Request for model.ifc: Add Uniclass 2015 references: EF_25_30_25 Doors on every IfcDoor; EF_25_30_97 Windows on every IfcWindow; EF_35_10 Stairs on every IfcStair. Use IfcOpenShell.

First a look at what the model holds.

```python
import ifcopenshell

model = ifcopenshell.open("model.ifc")
print(model.schema)
print("classifications:", [c.Name for c in model.by_type("IfcClassification")])
for ifc_class in ("IfcDoor", "IfcRoof", "IfcStair", "IfcWall", "IfcWindow"):
    print(ifc_class, len(model.by_type(ifc_class)))
```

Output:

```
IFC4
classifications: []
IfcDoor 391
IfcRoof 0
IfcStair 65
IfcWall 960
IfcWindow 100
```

```python
import ifcopenshell
import ifcopenshell.api.classification

model = ifcopenshell.open("model.ifc")

system = ifcopenshell.api.classification.add_classification(model, classification="Uniclass 2015")

codes = {
    "IfcDoor": ("EF_25_30_25", "Doors"),
    "IfcWindow": ("EF_25_30_97", "Windows"),
    "IfcStair": ("EF_35_10", "Stairs"),
}
for ifc_class, (code, name) in codes.items():
    products = model.by_type(ifc_class)
    ifcopenshell.api.classification.add_reference(
        model, products=products, classification=system, identification=code, name=name
    )
    print(code, len(products))

model.write("model_v2.ifc")
```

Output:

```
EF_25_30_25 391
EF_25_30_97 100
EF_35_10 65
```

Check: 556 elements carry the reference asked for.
